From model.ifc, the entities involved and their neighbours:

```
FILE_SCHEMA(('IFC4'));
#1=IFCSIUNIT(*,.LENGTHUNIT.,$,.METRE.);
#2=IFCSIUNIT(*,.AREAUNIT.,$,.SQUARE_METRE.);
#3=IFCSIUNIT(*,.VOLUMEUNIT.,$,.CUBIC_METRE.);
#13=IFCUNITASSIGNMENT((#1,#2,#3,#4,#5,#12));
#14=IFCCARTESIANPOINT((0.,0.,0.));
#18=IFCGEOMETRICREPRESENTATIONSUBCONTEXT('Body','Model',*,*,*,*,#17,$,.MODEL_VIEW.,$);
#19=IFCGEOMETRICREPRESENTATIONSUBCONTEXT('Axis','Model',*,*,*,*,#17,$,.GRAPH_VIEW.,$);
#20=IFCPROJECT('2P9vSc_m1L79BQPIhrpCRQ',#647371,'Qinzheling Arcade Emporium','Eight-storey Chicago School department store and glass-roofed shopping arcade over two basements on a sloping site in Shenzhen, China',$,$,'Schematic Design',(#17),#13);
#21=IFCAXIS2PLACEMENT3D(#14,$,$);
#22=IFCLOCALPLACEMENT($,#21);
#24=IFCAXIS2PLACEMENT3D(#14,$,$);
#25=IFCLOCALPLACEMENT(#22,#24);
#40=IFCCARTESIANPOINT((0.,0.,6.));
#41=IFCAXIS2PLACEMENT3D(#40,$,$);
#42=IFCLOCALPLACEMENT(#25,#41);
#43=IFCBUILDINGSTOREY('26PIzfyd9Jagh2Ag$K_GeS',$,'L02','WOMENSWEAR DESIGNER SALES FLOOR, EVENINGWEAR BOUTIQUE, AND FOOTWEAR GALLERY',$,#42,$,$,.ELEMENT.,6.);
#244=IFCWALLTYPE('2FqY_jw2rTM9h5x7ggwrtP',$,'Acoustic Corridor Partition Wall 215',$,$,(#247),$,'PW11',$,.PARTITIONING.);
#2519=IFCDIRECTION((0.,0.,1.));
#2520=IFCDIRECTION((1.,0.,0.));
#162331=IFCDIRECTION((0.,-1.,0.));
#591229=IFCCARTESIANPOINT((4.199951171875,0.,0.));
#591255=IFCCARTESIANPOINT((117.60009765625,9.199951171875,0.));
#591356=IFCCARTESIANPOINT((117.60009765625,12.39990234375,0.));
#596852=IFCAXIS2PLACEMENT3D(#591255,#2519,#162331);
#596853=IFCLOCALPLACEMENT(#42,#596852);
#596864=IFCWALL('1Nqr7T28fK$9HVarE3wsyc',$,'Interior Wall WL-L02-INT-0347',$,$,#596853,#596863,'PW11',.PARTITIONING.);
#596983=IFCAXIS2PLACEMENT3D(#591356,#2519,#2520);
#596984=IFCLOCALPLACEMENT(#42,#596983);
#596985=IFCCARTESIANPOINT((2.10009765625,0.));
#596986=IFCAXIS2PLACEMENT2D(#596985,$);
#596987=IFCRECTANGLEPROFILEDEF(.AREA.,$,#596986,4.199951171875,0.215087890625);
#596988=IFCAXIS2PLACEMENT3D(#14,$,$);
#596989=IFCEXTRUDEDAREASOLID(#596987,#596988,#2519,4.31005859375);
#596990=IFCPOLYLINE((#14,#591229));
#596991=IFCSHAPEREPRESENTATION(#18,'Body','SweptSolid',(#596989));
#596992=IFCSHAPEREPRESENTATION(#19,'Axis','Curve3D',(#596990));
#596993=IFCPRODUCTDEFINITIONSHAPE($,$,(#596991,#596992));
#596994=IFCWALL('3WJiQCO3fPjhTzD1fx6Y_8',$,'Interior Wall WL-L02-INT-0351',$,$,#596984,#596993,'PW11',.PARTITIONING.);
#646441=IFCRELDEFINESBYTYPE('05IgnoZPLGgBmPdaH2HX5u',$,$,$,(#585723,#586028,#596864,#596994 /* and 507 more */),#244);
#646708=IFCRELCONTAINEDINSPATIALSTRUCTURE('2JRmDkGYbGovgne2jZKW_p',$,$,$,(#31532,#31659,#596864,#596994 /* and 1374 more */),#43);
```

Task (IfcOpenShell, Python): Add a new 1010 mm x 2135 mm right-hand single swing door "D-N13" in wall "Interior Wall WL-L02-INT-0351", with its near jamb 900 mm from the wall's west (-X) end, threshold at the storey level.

```python
import numpy as np
import ifcopenshell
import ifcopenshell.api.feature
import ifcopenshell.api.geometry
import ifcopenshell.api.root
import ifcopenshell.api.spatial
import ifcopenshell.geom
import ifcopenshell.util.element
import ifcopenshell.util.placement
import ifcopenshell.util.representation
import ifcopenshell.util.shape
import ifcopenshell.util.unit

model = ifcopenshell.open("model.ifc")
unit_scale = ifcopenshell.util.unit.calculate_unit_scale(model)
settings = ifcopenshell.geom.settings()


def volume(element):
    """Net volume in cubic metres, openings subtracted."""
    shape = ifcopenshell.geom.create_shape(settings, element)
    return ifcopenshell.util.shape.get_volume(shape.geometry)


wall = model.by_guid("3WJiQCO3fPjhTzD1fx6Y_8")
storey = ifcopenshell.util.element.get_container(wall, ifc_class="IfcBuildingStorey")
context = ifcopenshell.util.representation.get_context(model, "Model", "Body", "MODEL_VIEW")
before = volume(wall)

width, height, from_end, sill = 1.01, 2.135, 0.9, 0.0  # metres

# The wall runs along its own X axis, and the end named is its -X end.
wall_shape = ifcopenshell.geom.create_shape(settings, wall)
x, y, z = ifcopenshell.util.shape.get_vertices(wall_shape.geometry).T
start = x.min() + from_end
face, thickness = float(y.min()), float(y.max() - y.min())
wall_matrix = ifcopenshell.util.placement.get_local_placement(wall.ObjectPlacement)
level = ifcopenshell.util.placement.get_local_placement(storey.ObjectPlacement)[2, 3]


def in_wall(x, y):
    """Placement at x, y metres in the wall's axes, at sill height."""
    matrix = wall_matrix.copy()
    matrix[:, 3] = wall_matrix @ np.array([x / unit_scale, y / unit_scale, 0.0, 1.0])
    matrix[2, 3] = level + sill / unit_scale
    return matrix


# Opening: a box that overshoots both wall faces by 50 mm.
opening = ifcopenshell.api.root.create_entity(model, ifc_class="IfcOpeningElement", predefined_type="OPENING")
box = ifcopenshell.api.geometry.add_wall_representation(
    model, context=context, length=width, height=height, thickness=thickness + 0.1
)
ifcopenshell.api.geometry.assign_representation(model, product=opening, representation=box)
ifcopenshell.api.geometry.edit_object_placement(model, product=opening, matrix=in_wall(start, face - 0.05), is_si=False)
ifcopenshell.api.feature.add_feature(model, feature=opening, element=wall)

door = ifcopenshell.api.root.create_entity(model, ifc_class="IfcDoor", name="D-N13", predefined_type="DOOR")
door.OverallWidth, door.OverallHeight = width / unit_scale, height / unit_scale
door.OperationType = "SINGLE_SWING_RIGHT"
body = ifcopenshell.api.geometry.add_door_representation(
    model,
    context=context,
    overall_width=door.OverallWidth,
    overall_height=door.OverallHeight,
    operation_type="SINGLE_SWING_RIGHT",
    lining_properties={"LiningDepth": thickness / unit_scale, "ThresholdDepth": thickness / unit_scale},
)
ifcopenshell.api.geometry.assign_representation(model, product=door, representation=body)
ifcopenshell.api.spatial.assign_container(model, products=[door], relating_structure=storey)
ifcopenshell.api.feature.add_filling(model, opening=opening, element=door)

# The lining spans the wall, so the door starts at the wall face.
ifcopenshell.api.geometry.edit_object_placement(model, product=door, matrix=in_wall(start, face), is_si=False)

after = volume(wall)

print(f"wall volume {before:.3f} -> {after:.3f} m3")

model.write("model_rev.ifc")
```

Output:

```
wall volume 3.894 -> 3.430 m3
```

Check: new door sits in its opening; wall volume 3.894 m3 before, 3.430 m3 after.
